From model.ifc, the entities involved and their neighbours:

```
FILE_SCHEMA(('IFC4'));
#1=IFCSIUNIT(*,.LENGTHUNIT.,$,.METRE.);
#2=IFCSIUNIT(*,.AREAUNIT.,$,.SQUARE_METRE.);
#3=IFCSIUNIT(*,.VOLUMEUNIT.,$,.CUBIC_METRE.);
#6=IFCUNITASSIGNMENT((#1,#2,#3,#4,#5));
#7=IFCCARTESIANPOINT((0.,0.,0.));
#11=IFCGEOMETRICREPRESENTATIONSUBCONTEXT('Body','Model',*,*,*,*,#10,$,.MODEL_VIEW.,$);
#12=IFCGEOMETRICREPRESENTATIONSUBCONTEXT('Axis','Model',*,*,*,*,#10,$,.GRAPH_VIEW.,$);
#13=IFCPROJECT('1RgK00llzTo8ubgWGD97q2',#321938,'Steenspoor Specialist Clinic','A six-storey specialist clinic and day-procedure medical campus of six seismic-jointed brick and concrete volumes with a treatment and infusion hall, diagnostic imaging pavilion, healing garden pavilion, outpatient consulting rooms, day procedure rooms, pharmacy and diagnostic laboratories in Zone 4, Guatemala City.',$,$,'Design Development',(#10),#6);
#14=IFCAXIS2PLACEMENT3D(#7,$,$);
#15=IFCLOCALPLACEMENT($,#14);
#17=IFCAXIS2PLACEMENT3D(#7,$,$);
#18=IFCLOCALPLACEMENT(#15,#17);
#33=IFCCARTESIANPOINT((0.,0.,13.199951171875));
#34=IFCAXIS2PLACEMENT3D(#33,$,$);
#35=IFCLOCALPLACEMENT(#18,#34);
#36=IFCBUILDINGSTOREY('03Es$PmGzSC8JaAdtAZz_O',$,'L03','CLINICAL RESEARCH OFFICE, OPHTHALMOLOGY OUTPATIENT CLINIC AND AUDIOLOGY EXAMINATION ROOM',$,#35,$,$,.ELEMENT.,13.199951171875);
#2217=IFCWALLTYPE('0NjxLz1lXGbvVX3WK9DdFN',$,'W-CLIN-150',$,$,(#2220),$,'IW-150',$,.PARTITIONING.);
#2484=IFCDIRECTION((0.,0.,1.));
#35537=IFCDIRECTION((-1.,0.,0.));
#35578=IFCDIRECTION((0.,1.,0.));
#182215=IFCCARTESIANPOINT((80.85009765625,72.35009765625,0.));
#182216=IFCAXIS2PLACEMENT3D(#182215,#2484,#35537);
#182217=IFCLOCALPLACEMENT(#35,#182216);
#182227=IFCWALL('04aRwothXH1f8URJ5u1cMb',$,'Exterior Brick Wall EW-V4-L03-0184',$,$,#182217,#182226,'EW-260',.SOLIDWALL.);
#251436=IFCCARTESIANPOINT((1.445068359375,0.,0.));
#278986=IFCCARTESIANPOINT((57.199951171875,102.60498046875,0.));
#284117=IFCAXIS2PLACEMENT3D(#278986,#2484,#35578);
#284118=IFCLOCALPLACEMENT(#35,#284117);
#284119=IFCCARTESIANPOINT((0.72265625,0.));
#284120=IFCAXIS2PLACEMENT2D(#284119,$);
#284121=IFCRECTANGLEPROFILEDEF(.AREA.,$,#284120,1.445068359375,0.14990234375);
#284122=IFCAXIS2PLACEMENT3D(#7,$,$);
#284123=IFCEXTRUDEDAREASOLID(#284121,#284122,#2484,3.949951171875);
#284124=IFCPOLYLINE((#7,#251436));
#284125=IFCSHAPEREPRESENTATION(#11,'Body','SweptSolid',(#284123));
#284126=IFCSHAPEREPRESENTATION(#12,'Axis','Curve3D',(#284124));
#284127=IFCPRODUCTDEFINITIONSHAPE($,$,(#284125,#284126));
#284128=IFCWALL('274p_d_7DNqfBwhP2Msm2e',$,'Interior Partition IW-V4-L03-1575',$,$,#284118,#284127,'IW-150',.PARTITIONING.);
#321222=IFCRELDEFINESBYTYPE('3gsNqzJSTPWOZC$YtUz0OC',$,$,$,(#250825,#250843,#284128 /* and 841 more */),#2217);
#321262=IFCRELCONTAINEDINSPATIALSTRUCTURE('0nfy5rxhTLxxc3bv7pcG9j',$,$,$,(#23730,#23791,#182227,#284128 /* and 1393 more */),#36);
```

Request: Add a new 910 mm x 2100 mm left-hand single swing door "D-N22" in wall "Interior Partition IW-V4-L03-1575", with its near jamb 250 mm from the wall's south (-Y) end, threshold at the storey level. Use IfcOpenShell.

```python
import numpy as np
import ifcopenshell
import ifcopenshell.api.feature
import ifcopenshell.api.geometry
import ifcopenshell.api.root
import ifcopenshell.api.spatial
import ifcopenshell.geom
import ifcopenshell.util.element
import ifcopenshell.util.placement
import ifcopenshell.util.representation
import ifcopenshell.util.shape
import ifcopenshell.util.unit

model = ifcopenshell.open("model.ifc")
unit_scale = ifcopenshell.util.unit.calculate_unit_scale(model)
settings = ifcopenshell.geom.settings()


def volume(element):
    """Net volume in cubic metres, openings subtracted."""
    shape = ifcopenshell.geom.create_shape(settings, element)
    return ifcopenshell.util.shape.get_volume(shape.geometry)


wall = model.by_guid("274p_d_7DNqfBwhP2Msm2e")
storey = ifcopenshell.util.element.get_container(wall, ifc_class="IfcBuildingStorey")
context = ifcopenshell.util.representation.get_context(model, "Model", "Body", "MODEL_VIEW")
before = volume(wall)

width, height, from_end, sill = 0.91, 2.1, 0.25, 0.0  # metres

# The wall runs along its own X axis, and the end named is its -X end.
wall_shape = ifcopenshell.geom.create_shape(settings, wall)
x, y, z = ifcopenshell.util.shape.get_vertices(wall_shape.geometry).T
start = x.min() + from_end
face, thickness = float(y.min()), float(y.max() - y.min())
wall_matrix = ifcopenshell.util.placement.get_local_placement(wall.ObjectPlacement)
level = ifcopenshell.util.placement.get_local_placement(storey.ObjectPlacement)[2, 3]


def in_wall(x, y):
    """Placement at x, y metres in the wall's axes, at sill height."""
    matrix = wall_matrix.copy()
    matrix[:, 3] = wall_matrix @ np.array([x / unit_scale, y / unit_scale, 0.0, 1.0])
    matrix[2, 3] = level + sill / unit_scale
    return matrix


# Opening: a box that overshoots both wall faces by 50 mm.
opening = ifcopenshell.api.root.create_entity(model, ifc_class="IfcOpeningElement", predefined_type="OPENING")
box = ifcopenshell.api.geometry.add_wall_representation(
    model, context=context, length=width, height=height, thickness=thickness + 0.1
)
ifcopenshell.api.geometry.assign_representation(model, product=opening, representation=box)
ifcopenshell.api.geometry.edit_object_placement(model, product=opening, matrix=in_wall(start, face - 0.05), is_si=False)
ifcopenshell.api.feature.add_feature(model, feature=opening, element=wall)

door = ifcopenshell.api.root.create_entity(model, ifc_class="IfcDoor", name="D-N22", predefined_type="DOOR")
door.OverallWidth, door.OverallHeight = width / unit_scale, height / unit_scale
door.OperationType = "SINGLE_SWING_LEFT"
body = ifcopenshell.api.geometry.add_door_representation(
    model,
    context=context,
    overall_width=door.OverallWidth,
    overall_height=door.OverallHeight,
    operation_type="SINGLE_SWING_LEFT",
    lining_properties={"LiningDepth": thickness / unit_scale, "ThresholdDepth": thickness / unit_scale},
)
ifcopenshell.api.geometry.assign_representation(model, product=door, representation=body)
ifcopenshell.api.spatial.assign_container(model, products=[door], relating_structure=storey)
ifcopenshell.api.feature.add_filling(model, opening=opening, element=door)

# The lining spans the wall, so the door starts at the wall face.
ifcopenshell.api.geometry.edit_object_placement(model, product=door, matrix=in_wall(start, face), is_si=False)

after = volume(wall)

print(f"wall volume {before:.3f} -> {after:.3f} m3")

model.write("model-out.ifc")
```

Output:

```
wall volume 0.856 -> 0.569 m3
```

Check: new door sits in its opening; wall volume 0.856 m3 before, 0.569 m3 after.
